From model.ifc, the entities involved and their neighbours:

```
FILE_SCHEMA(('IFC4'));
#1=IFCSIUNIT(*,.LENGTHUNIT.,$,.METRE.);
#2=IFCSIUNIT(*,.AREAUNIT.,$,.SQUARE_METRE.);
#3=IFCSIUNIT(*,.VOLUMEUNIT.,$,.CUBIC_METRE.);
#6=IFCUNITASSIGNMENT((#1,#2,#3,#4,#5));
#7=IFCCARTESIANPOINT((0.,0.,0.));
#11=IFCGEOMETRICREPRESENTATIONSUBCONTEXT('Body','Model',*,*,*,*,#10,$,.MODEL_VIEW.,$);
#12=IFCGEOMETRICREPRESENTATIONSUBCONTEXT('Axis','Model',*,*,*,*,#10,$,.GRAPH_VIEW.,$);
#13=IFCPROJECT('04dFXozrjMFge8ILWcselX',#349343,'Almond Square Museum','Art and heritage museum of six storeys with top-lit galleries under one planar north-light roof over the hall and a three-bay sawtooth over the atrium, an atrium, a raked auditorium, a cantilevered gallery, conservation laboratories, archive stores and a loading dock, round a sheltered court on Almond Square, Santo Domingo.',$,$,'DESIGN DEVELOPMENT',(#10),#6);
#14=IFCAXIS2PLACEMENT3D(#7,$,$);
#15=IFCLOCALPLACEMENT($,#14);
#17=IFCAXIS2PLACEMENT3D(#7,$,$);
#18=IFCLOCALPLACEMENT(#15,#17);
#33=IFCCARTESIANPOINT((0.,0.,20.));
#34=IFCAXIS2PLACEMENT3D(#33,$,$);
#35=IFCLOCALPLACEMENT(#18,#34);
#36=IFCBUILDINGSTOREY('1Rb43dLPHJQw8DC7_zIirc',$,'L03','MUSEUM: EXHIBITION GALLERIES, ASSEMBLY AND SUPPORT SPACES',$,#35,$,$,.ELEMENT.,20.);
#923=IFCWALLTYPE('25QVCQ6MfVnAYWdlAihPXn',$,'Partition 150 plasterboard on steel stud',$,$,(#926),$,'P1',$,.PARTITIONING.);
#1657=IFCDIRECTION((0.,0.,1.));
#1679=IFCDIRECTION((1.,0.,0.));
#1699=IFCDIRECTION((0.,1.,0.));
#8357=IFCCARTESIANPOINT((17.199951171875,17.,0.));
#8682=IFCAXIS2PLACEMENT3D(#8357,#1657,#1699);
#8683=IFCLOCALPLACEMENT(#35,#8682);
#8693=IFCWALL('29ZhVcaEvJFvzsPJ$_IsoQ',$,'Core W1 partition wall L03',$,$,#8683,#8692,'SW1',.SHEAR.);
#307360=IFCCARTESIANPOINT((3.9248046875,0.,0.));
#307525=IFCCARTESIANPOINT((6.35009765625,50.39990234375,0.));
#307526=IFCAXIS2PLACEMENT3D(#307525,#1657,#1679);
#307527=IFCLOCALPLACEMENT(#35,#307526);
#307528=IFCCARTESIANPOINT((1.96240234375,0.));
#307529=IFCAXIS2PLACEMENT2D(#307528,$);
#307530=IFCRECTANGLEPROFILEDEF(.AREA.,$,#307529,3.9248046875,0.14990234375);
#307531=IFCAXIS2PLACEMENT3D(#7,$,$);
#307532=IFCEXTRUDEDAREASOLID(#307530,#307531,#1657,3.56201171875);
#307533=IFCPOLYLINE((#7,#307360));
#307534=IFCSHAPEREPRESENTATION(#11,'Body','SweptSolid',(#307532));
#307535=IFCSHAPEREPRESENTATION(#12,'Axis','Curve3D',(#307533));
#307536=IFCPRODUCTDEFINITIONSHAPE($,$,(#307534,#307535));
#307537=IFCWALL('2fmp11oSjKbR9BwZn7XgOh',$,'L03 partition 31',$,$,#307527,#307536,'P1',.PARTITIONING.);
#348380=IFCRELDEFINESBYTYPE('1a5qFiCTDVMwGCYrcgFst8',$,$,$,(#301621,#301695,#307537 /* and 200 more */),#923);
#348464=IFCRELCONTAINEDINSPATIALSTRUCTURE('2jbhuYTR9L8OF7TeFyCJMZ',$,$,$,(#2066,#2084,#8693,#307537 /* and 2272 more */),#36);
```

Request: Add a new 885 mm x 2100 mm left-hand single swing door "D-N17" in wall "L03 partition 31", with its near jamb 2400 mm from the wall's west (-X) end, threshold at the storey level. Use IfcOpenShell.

```python
import numpy as np
import ifcopenshell
import ifcopenshell.api.feature
import ifcopenshell.api.geometry
import ifcopenshell.api.root
import ifcopenshell.api.spatial
import ifcopenshell.geom
import ifcopenshell.util.element
import ifcopenshell.util.placement
import ifcopenshell.util.representation
import ifcopenshell.util.shape
import ifcopenshell.util.unit

model = ifcopenshell.open("model.ifc")
unit_scale = ifcopenshell.util.unit.calculate_unit_scale(model)
settings = ifcopenshell.geom.settings()


def volume(element):
    """Net volume in cubic metres, openings subtracted."""
    shape = ifcopenshell.geom.create_shape(settings, element)
    return ifcopenshell.util.shape.get_volume(shape.geometry)


wall = model.by_guid("2fmp11oSjKbR9BwZn7XgOh")
storey = ifcopenshell.util.element.get_container(wall, ifc_class="IfcBuildingStorey")
context = ifcopenshell.util.representation.get_context(model, "Model", "Body", "MODEL_VIEW")
before = volume(wall)

width, height, from_end, sill = 0.885, 2.1, 2.4, 0.0  # metres

# The wall runs along its own X axis, and the end named is its -X end.
wall_shape = ifcopenshell.geom.create_shape(settings, wall)
x, y, z = ifcopenshell.util.shape.get_vertices(wall_shape.geometry).T
start = x.min() + from_end
face, thickness = float(y.min()), float(y.max() - y.min())
wall_matrix = ifcopenshell.util.placement.get_local_placement(wall.ObjectPlacement)
level = ifcopenshell.util.placement.get_local_placement(storey.ObjectPlacement)[2, 3]


def in_wall(x, y):
    """Placement at x, y metres in the wall's axes, at sill height."""
    matrix = wall_matrix.copy()
    matrix[:, 3] = wall_matrix @ np.array([x / unit_scale, y / unit_scale, 0.0, 1.0])
    matrix[2, 3] = level + sill / unit_scale
    return matrix


# Opening: a box that overshoots both wall faces by 50 mm.
opening = ifcopenshell.api.root.create_entity(model, ifc_class="IfcOpeningElement", predefined_type="OPENING")
box = ifcopenshell.api.geometry.add_wall_representation(
    model, context=context, length=width, height=height, thickness=thickness + 0.1
)
ifcopenshell.api.geometry.assign_representation(model, product=opening, representation=box)
ifcopenshell.api.geometry.edit_object_placement(model, product=opening, matrix=in_wall(start, face - 0.05), is_si=False)
ifcopenshell.api.feature.add_feature(model, feature=opening, element=wall)

door = ifcopenshell.api.root.create_entity(model, ifc_class="IfcDoor", name="D-N17", predefined_type="DOOR")
door.OverallWidth, door.OverallHeight = width / unit_scale, height / unit_scale
door.OperationType = "SINGLE_SWING_LEFT"
body = ifcopenshell.api.geometry.add_door_representation(
    model,
    context=context,
    overall_width=door.OverallWidth,
    overall_height=door.OverallHeight,
    operation_type="SINGLE_SWING_LEFT",
    lining_properties={"LiningDepth": thickness / unit_scale, "ThresholdDepth": thickness / unit_scale},
)
ifcopenshell.api.geometry.assign_representation(model, product=door, representation=body)
ifcopenshell.api.spatial.assign_container(model, products=[door], relating_structure=storey)
ifcopenshell.api.feature.add_filling(model, opening=opening, element=door)

# The lining spans the wall, so the door starts at the wall face.
ifcopenshell.api.geometry.edit_object_placement(model, product=door, matrix=in_wall(start, face), is_si=False)

after = volume(wall)

print(f"wall volume {before:.3f} -> {after:.3f} m3")

model.write("model_v2.ifc")
```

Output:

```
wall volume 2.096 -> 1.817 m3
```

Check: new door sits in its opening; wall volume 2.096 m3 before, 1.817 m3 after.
